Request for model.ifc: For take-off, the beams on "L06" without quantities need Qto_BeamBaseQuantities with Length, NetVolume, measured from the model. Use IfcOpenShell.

First a look at what the model holds.

```python
import ifcopenshell
import ifcopenshell.util.element
import ifcopenshell.util.unit

model = ifcopenshell.open("model.ifc")
print(model.schema)
for unit_type in ("LENGTHUNIT", "AREAUNIT", "VOLUMEUNIT"):
    print(unit_type, ifcopenshell.util.unit.calculate_unit_scale(model, unit_type))
storey = next(s for s in model.by_type("IfcBuildingStorey") if s.Name == "L06")
beams = [e for e in ifcopenshell.util.element.get_decomposition(storey) if e.is_a("IfcBeam")]
for e in sorted(beams, key=lambda e: e.id()):
    print(e.id(), e.is_a(), e.Name, list(ifcopenshell.util.element.get_psets(e, qtos_only=True)), sep=" | ")
```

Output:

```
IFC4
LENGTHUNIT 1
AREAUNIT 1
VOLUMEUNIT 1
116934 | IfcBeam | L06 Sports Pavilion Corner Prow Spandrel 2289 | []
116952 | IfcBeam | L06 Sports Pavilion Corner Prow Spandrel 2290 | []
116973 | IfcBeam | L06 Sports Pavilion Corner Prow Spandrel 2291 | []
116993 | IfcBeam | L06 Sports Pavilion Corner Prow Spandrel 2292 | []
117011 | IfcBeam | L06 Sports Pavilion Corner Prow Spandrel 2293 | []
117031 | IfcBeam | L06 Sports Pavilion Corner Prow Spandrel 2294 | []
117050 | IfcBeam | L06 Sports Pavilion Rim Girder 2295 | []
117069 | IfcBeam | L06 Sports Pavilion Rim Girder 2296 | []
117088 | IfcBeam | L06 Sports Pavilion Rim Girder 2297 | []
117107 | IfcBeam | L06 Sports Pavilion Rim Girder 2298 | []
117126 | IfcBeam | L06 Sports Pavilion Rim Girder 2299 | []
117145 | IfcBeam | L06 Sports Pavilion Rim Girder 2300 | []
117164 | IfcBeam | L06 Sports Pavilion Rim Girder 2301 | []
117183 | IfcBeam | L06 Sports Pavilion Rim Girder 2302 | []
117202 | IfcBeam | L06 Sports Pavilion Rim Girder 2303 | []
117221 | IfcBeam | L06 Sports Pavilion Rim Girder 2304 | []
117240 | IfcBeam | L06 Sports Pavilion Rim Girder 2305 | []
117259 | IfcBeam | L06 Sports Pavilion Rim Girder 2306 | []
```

```python
import ifcopenshell
import ifcopenshell.api.pset
import ifcopenshell.geom
import ifcopenshell.util.element
import ifcopenshell.util.shape
import ifcopenshell.util.unit

model = ifcopenshell.open("model.ifc")
unit_scale = ifcopenshell.util.unit.calculate_unit_scale(model)
volume_scale = ifcopenshell.util.unit.calculate_unit_scale(model, "VOLUMEUNIT")
settings = ifcopenshell.geom.settings()

storey = next(s for s in model.by_type("IfcBuildingStorey") if s.Name == "L06")
beams = [e for e in ifcopenshell.util.element.get_decomposition(storey) if e.is_a("IfcBeam")]

for e in sorted(beams, key=lambda e: e.id()):
    if ifcopenshell.util.element.get_psets(e, qtos_only=True, should_inherit=False):
        continue
    # Geometry comes back in metres, in the element's own axes.
    shape = ifcopenshell.geom.create_shape(settings, e)
    values = {
        "Length": ifcopenshell.util.shape.get_max_xyz(shape.geometry) / unit_scale,
        "NetVolume": ifcopenshell.util.shape.get_volume(shape.geometry) / volume_scale,
    }
    qto = ifcopenshell.api.pset.add_qto(model, product=e, name="Qto_BeamBaseQuantities")
    ifcopenshell.api.pset.edit_qto(model, qto=qto, properties=values)
    print(e.id(), {k: round(v, 3) for k, v in values.items()})

model.write("model-out.ifc")
```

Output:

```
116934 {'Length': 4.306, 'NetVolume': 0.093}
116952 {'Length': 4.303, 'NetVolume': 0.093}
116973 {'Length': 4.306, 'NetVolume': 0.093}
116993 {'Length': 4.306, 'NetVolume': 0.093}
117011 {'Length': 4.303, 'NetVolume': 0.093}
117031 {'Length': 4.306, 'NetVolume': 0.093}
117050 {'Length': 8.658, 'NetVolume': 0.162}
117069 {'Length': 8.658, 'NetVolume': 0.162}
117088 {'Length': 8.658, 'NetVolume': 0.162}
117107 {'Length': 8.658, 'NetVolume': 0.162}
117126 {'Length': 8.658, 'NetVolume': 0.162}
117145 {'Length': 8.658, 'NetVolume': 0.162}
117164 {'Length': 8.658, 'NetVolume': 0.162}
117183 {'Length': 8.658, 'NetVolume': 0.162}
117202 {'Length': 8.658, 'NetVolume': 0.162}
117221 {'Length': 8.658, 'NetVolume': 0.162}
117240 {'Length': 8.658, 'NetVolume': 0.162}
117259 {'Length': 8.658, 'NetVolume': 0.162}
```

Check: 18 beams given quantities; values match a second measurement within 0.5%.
